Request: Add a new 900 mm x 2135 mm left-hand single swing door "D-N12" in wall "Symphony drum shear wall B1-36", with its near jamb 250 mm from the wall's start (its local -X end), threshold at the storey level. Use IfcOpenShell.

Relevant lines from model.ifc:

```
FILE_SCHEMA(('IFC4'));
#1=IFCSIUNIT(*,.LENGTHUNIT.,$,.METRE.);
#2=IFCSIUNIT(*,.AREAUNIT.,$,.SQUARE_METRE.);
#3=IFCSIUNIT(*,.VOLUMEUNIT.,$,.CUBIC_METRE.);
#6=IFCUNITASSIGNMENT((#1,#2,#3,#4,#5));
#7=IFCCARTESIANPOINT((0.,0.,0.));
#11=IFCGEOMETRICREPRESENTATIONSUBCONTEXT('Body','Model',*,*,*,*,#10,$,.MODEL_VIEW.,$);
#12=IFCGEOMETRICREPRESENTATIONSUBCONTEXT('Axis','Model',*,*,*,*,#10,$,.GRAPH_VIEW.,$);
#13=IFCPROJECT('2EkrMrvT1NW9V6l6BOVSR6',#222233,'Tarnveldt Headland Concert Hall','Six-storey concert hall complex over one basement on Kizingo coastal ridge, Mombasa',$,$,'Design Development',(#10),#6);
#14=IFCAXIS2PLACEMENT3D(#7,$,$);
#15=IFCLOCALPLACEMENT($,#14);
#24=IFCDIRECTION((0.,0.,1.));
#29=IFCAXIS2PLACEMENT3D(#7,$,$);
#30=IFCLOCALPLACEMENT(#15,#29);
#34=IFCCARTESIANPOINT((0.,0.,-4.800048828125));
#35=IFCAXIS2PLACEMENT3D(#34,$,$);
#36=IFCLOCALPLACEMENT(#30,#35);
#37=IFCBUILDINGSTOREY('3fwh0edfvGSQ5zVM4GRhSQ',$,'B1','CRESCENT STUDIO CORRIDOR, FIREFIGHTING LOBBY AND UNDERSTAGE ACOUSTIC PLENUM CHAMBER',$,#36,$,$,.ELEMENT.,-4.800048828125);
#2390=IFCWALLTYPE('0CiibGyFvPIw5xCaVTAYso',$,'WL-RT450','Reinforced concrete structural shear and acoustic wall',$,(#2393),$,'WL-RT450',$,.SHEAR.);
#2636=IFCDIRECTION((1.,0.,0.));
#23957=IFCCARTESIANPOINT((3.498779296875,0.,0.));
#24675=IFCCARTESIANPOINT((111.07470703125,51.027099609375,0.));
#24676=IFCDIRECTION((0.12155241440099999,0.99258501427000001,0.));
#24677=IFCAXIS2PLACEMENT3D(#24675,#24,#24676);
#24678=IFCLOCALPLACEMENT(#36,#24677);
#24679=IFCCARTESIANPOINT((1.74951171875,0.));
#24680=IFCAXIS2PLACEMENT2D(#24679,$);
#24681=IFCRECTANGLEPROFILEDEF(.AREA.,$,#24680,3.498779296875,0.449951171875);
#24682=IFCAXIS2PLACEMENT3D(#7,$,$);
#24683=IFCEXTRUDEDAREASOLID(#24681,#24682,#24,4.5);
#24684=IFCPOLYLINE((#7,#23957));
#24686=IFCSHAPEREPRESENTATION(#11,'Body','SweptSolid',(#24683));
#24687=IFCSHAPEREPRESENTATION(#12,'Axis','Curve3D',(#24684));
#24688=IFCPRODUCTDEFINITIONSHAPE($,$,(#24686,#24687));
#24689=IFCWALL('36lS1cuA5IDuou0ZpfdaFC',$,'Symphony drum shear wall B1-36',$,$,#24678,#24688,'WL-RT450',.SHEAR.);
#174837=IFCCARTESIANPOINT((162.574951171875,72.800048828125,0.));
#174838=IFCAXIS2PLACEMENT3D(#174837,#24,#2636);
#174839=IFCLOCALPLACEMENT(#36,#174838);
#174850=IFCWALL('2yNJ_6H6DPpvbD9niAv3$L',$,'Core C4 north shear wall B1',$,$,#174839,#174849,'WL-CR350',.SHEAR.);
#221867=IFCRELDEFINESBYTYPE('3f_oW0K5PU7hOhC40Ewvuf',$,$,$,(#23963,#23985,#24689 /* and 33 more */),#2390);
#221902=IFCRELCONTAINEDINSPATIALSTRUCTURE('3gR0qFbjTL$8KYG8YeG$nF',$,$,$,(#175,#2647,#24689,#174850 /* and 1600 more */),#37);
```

```python
import numpy as np
import ifcopenshell
import ifcopenshell.api.feature
import ifcopenshell.api.geometry
import ifcopenshell.api.root
import ifcopenshell.api.spatial
import ifcopenshell.geom
import ifcopenshell.util.element
import ifcopenshell.util.placement
import ifcopenshell.util.representation
import ifcopenshell.util.shape
import ifcopenshell.util.unit

model = ifcopenshell.open("model.ifc")
unit_scale = ifcopenshell.util.unit.calculate_unit_scale(model)
settings = ifcopenshell.geom.settings()


def volume(element):
    """Net volume in cubic metres, openings subtracted."""
    shape = ifcopenshell.geom.create_shape(settings, element)
    return ifcopenshell.util.shape.get_volume(shape.geometry)


wall = model.by_id(24689)
storey = ifcopenshell.util.element.get_container(wall, ifc_class="IfcBuildingStorey")
context = ifcopenshell.util.representation.get_context(model, "Model", "Body", "MODEL_VIEW")
before = volume(wall)

width, height, from_end, sill = 0.9, 2.135, 0.25, 0.0  # metres

# The wall runs along its own X axis, and the end named is its -X end.
wall_shape = ifcopenshell.geom.create_shape(settings, wall)
x, y, z = ifcopenshell.util.shape.get_vertices(wall_shape.geometry).T
start = x.min() + from_end
face, thickness = float(y.min()), float(y.max() - y.min())
wall_matrix = ifcopenshell.util.placement.get_local_placement(wall.ObjectPlacement)
level = ifcopenshell.util.placement.get_local_placement(storey.ObjectPlacement)[2, 3]


def in_wall(x, y):
    """Placement at x, y metres in the wall's axes, at sill height."""
    matrix = wall_matrix.copy()
    matrix[:, 3] = wall_matrix @ np.array([x / unit_scale, y / unit_scale, 0.0, 1.0])
    matrix[2, 3] = level + sill / unit_scale
    return matrix


# Opening: a box that overshoots both wall faces by 50 mm.
opening = ifcopenshell.api.root.create_entity(model, ifc_class="IfcOpeningElement", predefined_type="OPENING")
box = ifcopenshell.api.geometry.add_wall_representation(
    model, context=context, length=width, height=height, thickness=thickness + 0.1
)
ifcopenshell.api.geometry.assign_representation(model, product=opening, representation=box)
ifcopenshell.api.geometry.edit_object_placement(model, product=opening, matrix=in_wall(start, face - 0.05), is_si=False)
ifcopenshell.api.feature.add_feature(model, feature=opening, element=wall)

door = ifcopenshell.api.root.create_entity(model, ifc_class="IfcDoor", name="D-N12", predefined_type="DOOR")
door.OverallWidth, door.OverallHeight = width / unit_scale, height / unit_scale
door.OperationType = "SINGLE_SWING_LEFT"
body = ifcopenshell.api.geometry.add_door_representation(
    model,
    context=context,
    overall_width=door.OverallWidth,
    overall_height=door.OverallHeight,
    operation_type="SINGLE_SWING_LEFT",
    lining_properties={"LiningDepth": thickness / unit_scale, "ThresholdDepth": thickness / unit_scale},
)
ifcopenshell.api.geometry.assign_representation(model, product=door, representation=body)
ifcopenshell.api.spatial.assign_container(model, products=[door], relating_structure=storey)
ifcopenshell.api.feature.add_filling(model, opening=opening, element=door)

# The lining spans the wall, so the door starts at the wall face.
ifcopenshell.api.geometry.edit_object_placement(model, product=door, matrix=in_wall(start, face), is_si=False)

after = volume(wall)

print(f"wall volume {before:.3f} -> {after:.3f} m3")

model.write("model_rev.ifc")
```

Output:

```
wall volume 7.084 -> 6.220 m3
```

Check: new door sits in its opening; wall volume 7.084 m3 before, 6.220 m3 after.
